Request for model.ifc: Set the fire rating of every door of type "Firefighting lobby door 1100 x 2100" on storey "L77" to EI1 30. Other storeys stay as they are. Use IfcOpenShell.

First a look at what the model holds.

```python
import ifcopenshell
import ifcopenshell.util.element

model = ifcopenshell.open("model.ifc")
print(model.schema)
storey = next(s for s in model.by_type("IfcBuildingStorey") if s.Name == "L77")
doors = [e for e in ifcopenshell.util.element.get_decomposition(storey) if e.is_a("IfcDoor")]
seen = {}
for e in doors:
    element_type = ifcopenshell.util.element.get_type(e)
    key = (element_type.Name if element_type != e and element_type else None, ifcopenshell.util.element.get_pset(e, "Pset_DoorCommon", "FireRating"))
    seen[key] = seen.get(key, 0) + 1
for (name, value), count in sorted(seen.items(), key=str):
    print(count, "x", name, "|", value)
```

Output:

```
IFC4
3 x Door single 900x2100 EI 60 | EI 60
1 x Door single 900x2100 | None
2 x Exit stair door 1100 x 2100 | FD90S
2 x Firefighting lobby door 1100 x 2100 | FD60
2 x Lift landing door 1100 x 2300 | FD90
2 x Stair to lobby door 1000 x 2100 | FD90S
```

```python
import ifcopenshell
import ifcopenshell.api.pset
import ifcopenshell.util.element

model = ifcopenshell.open("model.ifc")

storey = next(s for s in model.by_type("IfcBuildingStorey") if s.Name == "L77")
doors = [e for e in ifcopenshell.util.element.get_decomposition(storey) if e.is_a("IfcDoor")]

count = 0
for e in doors:
    element_type = ifcopenshell.util.element.get_type(e)
    if element_type in (None, e) or element_type.Name != "Firefighting lobby door 1100 x 2100":
        continue
    found = ifcopenshell.util.element.get_pset(e, "Pset_DoorCommon", should_inherit=False)
    if found:
        pset = model.by_id(found["id"])
        if len(ifcopenshell.util.element.get_elements_by_pset(pset)) > 1:
            pset = ifcopenshell.api.pset.unshare_pset(model, products=[e], pset=pset)[0]
    else:
        pset = ifcopenshell.api.pset.add_pset(model, product=e, name="Pset_DoorCommon")
    ifcopenshell.api.pset.edit_pset(model, pset=pset, properties={"FireRating": "EI1 30"})
    count += 1

print(count, "doors updated")

model.write("model_rev.ifc")
```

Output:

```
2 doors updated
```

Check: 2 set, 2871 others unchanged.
